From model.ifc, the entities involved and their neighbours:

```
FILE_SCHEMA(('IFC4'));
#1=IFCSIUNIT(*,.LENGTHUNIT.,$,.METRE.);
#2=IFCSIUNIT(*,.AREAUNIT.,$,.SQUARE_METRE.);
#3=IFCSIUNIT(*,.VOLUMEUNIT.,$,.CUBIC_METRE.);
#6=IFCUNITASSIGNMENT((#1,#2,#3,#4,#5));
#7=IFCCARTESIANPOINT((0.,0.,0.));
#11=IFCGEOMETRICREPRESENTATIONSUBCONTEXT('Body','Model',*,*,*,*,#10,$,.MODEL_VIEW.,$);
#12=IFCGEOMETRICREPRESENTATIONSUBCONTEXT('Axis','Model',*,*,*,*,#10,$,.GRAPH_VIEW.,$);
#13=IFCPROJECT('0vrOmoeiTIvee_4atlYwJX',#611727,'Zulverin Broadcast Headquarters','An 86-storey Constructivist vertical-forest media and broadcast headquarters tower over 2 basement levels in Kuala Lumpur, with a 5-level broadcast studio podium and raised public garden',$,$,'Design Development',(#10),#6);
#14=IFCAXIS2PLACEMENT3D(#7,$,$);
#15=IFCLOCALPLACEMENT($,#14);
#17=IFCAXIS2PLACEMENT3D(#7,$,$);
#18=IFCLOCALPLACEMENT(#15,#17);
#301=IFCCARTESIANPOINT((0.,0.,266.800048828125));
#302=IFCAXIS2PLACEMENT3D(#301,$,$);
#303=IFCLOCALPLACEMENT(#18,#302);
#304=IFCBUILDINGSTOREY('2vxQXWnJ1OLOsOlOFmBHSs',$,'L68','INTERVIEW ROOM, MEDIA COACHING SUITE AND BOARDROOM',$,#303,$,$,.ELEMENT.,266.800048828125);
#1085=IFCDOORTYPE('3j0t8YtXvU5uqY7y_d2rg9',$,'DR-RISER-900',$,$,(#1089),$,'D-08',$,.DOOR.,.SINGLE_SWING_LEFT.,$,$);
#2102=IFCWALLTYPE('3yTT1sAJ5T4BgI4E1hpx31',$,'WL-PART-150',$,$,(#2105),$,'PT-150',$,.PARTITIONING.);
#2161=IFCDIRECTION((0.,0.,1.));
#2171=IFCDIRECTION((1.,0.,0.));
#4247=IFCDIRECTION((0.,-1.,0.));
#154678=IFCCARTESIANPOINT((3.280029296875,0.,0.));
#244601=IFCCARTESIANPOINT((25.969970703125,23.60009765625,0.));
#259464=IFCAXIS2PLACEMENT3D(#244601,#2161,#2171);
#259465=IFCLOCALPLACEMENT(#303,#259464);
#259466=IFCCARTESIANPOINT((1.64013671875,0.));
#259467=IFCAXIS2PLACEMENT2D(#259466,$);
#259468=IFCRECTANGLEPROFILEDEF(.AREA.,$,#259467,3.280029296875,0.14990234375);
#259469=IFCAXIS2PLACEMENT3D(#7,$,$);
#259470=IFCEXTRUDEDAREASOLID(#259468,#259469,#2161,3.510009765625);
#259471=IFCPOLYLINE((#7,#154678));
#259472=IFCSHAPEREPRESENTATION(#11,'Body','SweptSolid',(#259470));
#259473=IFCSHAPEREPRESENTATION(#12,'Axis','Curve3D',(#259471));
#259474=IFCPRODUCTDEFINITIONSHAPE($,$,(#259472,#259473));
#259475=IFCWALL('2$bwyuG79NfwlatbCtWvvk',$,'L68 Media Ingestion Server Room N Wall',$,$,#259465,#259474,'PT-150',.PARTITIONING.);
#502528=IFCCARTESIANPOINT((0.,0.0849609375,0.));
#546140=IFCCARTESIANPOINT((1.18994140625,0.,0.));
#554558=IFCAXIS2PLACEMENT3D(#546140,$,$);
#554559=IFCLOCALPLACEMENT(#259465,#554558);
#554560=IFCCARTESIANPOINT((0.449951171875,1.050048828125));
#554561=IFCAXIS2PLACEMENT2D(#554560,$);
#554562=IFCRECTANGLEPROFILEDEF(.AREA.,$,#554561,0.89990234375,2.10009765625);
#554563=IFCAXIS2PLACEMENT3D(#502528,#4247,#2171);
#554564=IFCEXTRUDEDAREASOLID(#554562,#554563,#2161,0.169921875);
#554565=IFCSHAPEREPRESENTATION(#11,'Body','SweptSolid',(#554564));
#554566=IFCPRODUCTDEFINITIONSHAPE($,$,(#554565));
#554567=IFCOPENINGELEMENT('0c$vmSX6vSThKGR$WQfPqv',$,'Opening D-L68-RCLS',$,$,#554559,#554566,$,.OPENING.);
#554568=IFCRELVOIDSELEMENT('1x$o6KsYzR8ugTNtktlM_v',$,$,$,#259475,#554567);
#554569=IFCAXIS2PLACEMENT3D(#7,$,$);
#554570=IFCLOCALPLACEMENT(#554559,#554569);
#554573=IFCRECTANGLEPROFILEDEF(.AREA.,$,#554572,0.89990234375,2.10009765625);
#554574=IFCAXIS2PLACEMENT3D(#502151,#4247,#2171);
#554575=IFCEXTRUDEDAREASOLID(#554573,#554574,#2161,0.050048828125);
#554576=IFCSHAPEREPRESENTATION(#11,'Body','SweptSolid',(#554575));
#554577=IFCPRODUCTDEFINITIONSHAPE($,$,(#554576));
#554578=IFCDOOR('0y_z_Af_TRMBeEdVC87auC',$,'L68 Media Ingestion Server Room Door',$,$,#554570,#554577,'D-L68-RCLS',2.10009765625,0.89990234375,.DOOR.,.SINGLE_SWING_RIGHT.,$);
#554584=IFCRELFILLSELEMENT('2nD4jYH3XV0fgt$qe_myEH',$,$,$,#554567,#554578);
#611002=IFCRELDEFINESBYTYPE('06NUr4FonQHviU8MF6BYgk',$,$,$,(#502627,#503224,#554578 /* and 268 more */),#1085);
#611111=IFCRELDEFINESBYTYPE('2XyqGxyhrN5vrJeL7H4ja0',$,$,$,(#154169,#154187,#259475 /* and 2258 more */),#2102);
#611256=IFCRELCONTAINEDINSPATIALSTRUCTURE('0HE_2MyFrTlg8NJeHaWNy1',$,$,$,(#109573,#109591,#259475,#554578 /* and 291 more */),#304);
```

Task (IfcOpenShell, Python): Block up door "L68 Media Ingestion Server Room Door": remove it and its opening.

```python
import ifcopenshell
import ifcopenshell.api.feature
import ifcopenshell.api.root
import ifcopenshell.geom
import ifcopenshell.util.shape

model = ifcopenshell.open("model.ifc")
settings = ifcopenshell.geom.settings()


def volume(element):
    """Net volume in cubic metres, openings subtracted."""
    shape = ifcopenshell.geom.create_shape(settings, element)
    return ifcopenshell.util.shape.get_volume(shape.geometry)


door = model.by_id(554578)
opening = door.FillsVoids[0].RelatingOpeningElement
wall = opening.VoidsElements[0].RelatingBuildingElement
before = volume(wall)

ifcopenshell.api.root.remove_product(model, product=door)
ifcopenshell.api.feature.remove_feature(model, feature=opening)

after = volume(wall)

print(f"wall volume {before:.3f} -> {after:.3f} m3")

model.write("model-out.ifc")
```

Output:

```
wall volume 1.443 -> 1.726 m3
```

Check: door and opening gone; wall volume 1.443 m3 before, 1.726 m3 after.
